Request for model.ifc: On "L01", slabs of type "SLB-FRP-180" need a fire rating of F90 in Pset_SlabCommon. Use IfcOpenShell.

First a look at what the model holds.

```python
import ifcopenshell
import ifcopenshell.util.element

model = ifcopenshell.open("model.ifc")
print(model.schema)
storey = next(s for s in model.by_type("IfcBuildingStorey") if s.Name == "L01")
slabs = [e for e in ifcopenshell.util.element.get_decomposition(storey) if e.is_a("IfcSlab")]
seen = {}
for e in slabs:
    element_type = ifcopenshell.util.element.get_type(e)
    key = (element_type.Name if element_type != e and element_type else None, ifcopenshell.util.element.get_pset(e, "Pset_SlabCommon", "FireRating"))
    seen[key] = seen.get(key, 0) + 1
for (name, value), count in sorted(seen.items(), key=str):
    print(count, "x", name, "|", value)
```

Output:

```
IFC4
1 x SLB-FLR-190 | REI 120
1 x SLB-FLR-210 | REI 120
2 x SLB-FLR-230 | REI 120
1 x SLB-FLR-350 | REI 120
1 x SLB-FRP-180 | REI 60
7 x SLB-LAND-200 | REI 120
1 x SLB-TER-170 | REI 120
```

```python
import ifcopenshell
import ifcopenshell.api.pset
import ifcopenshell.util.element

model = ifcopenshell.open("model.ifc")

storey = next(s for s in model.by_type("IfcBuildingStorey") if s.Name == "L01")
slabs = [e for e in ifcopenshell.util.element.get_decomposition(storey) if e.is_a("IfcSlab")]

count = 0
for e in slabs:
    element_type = ifcopenshell.util.element.get_type(e)
    if element_type in (None, e) or element_type.Name != "SLB-FRP-180":
        continue
    # add_pset returns the element's existing set when there is one.
    pset = ifcopenshell.api.pset.add_pset(model, product=e, name="Pset_SlabCommon")
    ifcopenshell.api.pset.edit_pset(model, pset=pset, properties={"FireRating": "F90"})
    count += 1

print(count, "slabs updated")

model.write("model_edited.ifc")
```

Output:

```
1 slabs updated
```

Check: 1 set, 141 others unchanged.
